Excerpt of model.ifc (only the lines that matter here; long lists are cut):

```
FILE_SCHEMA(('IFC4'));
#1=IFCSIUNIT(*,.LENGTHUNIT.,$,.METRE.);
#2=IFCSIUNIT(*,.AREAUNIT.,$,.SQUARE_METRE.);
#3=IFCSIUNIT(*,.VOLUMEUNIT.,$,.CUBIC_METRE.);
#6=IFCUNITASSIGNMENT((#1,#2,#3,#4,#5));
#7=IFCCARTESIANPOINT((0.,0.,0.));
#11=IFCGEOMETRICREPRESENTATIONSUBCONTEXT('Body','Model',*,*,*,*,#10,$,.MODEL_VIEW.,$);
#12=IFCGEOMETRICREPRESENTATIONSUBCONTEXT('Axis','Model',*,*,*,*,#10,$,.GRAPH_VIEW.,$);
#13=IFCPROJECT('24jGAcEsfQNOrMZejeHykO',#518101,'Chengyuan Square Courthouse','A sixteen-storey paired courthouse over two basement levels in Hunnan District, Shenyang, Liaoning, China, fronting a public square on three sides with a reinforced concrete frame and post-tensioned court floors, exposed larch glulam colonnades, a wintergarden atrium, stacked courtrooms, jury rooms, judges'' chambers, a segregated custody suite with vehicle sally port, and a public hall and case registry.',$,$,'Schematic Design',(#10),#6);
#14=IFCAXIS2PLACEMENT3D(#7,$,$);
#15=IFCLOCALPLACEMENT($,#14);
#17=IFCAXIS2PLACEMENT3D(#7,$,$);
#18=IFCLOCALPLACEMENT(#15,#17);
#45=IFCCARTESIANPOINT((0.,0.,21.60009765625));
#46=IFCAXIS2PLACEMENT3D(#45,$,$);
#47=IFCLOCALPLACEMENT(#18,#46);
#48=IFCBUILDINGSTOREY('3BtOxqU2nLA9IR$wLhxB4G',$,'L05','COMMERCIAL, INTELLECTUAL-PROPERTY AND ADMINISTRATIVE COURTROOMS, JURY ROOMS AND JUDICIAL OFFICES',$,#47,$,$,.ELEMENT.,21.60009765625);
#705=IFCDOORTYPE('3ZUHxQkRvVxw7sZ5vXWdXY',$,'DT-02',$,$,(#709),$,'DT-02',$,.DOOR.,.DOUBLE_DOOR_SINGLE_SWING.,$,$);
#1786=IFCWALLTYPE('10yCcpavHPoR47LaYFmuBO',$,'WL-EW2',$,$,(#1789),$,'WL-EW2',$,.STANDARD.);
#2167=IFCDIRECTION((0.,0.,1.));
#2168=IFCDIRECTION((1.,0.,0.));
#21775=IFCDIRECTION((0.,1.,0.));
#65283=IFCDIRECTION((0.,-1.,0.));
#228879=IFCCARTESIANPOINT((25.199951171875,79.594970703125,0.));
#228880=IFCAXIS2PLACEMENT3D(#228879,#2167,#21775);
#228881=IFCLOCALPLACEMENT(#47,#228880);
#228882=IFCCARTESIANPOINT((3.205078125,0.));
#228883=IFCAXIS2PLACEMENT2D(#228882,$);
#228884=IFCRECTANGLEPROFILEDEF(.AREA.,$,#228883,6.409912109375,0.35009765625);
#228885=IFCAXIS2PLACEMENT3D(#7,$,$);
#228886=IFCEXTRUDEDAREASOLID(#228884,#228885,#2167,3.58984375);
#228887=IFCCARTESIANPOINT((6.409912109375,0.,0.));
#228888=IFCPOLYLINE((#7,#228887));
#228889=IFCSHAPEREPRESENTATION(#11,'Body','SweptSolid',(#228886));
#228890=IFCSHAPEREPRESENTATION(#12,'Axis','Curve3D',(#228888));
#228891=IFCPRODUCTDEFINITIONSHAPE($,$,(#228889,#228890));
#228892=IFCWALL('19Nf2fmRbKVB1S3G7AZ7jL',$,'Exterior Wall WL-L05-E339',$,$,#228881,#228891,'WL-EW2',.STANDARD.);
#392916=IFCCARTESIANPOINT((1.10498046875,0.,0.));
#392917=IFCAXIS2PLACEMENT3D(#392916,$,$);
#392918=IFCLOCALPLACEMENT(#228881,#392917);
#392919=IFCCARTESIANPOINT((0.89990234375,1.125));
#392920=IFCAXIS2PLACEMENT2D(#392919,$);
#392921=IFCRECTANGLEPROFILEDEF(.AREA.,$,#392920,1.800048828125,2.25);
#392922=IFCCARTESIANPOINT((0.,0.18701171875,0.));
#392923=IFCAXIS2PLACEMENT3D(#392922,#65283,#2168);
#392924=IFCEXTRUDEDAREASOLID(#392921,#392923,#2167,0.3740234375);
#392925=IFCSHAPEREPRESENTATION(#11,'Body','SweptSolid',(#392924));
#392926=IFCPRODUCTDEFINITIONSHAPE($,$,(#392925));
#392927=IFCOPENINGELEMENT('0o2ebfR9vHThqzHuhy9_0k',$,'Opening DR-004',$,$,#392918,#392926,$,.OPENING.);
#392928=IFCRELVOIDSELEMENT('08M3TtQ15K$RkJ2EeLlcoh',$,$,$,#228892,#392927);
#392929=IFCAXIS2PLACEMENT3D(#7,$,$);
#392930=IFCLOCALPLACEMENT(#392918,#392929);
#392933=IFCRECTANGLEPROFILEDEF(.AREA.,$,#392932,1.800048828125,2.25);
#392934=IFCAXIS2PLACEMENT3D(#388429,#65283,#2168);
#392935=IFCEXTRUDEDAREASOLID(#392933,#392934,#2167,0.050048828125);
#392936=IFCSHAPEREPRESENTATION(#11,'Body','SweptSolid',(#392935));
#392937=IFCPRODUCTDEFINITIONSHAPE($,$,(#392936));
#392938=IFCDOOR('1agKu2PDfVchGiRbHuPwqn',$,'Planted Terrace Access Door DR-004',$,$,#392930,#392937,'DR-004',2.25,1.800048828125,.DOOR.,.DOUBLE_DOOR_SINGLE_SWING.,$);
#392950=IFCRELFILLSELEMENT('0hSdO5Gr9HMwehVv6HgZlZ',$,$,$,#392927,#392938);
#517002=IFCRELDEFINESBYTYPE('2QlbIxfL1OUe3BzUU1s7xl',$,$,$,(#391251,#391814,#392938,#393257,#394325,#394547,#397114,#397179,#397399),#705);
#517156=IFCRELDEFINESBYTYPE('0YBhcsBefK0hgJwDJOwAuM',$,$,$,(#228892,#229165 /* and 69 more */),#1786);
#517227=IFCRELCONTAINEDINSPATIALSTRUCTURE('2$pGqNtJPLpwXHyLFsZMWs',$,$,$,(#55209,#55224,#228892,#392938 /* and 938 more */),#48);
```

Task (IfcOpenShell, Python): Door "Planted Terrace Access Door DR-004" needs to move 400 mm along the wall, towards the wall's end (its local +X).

```python
import ifcopenshell
import ifcopenshell.api.geometry
import ifcopenshell.util.placement
import ifcopenshell.util.unit

model = ifcopenshell.open("model.ifc")
unit_scale = ifcopenshell.util.unit.calculate_unit_scale(model)

door = model.by_id(392938)
opening = door.FillsVoids[0].RelatingOpeningElement
wall = opening.VoidsElements[0].RelatingBuildingElement

wall_matrix = ifcopenshell.util.placement.get_local_placement(wall.ObjectPlacement)
shift = wall_matrix[:3, 0] * 0.4 / unit_scale
before = ifcopenshell.util.placement.get_local_placement(door.ObjectPlacement)[:3, 3].copy()

# The door is placed relative to its opening, so it follows when the opening moves.
matrix = ifcopenshell.util.placement.get_local_placement(opening.ObjectPlacement)
matrix[:3, 3] += shift
ifcopenshell.api.geometry.edit_object_placement(
    model, product=opening, matrix=matrix, is_si=False, should_transform_children=True
)

after = ifcopenshell.util.placement.get_local_placement(door.ObjectPlacement)[:3, 3]
print("door moved by", (after - before).round(3) + 0.0)

model.write("model_updated.ifc")
```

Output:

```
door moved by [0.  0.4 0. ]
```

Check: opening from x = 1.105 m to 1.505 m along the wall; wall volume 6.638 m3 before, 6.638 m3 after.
